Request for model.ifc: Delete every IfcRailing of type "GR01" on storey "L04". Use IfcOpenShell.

First a look at what the model holds.

```python
import ifcopenshell
import ifcopenshell.util.element

model = ifcopenshell.open("model.ifc")
print(model.schema)
storey = next(s for s in model.by_type("IfcBuildingStorey") if s.Name == "L04")
railings = [e for e in ifcopenshell.util.element.get_decomposition(storey) if e.is_a("IfcRailing")]
seen = {}
for e in railings:
    element_type = ifcopenshell.util.element.get_type(e)
    name = element_type.Name if element_type not in (None, e) else None
    seen[name] = seen.get(name, 0) + 1
for name, count in sorted(seen.items(), key=str):
    print(count, "x", name)
```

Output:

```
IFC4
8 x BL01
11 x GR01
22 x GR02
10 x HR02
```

```python
import ifcopenshell
import ifcopenshell.api.root
import ifcopenshell.util.element

model = ifcopenshell.open("model.ifc")

storey = next(s for s in model.by_type("IfcBuildingStorey") if s.Name == "L04")
railings = [e for e in ifcopenshell.util.element.get_decomposition(storey) if e.is_a("IfcRailing")]
targets = [e for e in railings if (t := ifcopenshell.util.element.get_type(e)) not in (None, e) and t.Name == "GR01"]

for e in targets:
    ifcopenshell.api.root.remove_product(model, product=e)
print(len(targets), "removed")

model.write("model_edited.ifc")
```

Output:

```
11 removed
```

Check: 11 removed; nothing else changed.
